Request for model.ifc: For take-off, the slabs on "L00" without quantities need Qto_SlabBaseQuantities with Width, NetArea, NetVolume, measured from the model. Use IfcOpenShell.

First a look at what the model holds.

```python
import ifcopenshell
import ifcopenshell.util.element
import ifcopenshell.util.unit

model = ifcopenshell.open("model.ifc")
print(model.schema)
for unit_type in ("LENGTHUNIT", "AREAUNIT", "VOLUMEUNIT"):
    print(unit_type, ifcopenshell.util.unit.calculate_unit_scale(model, unit_type))
storey = next(s for s in model.by_type("IfcBuildingStorey") if s.Name == "L00")
slabs = [e for e in ifcopenshell.util.element.get_decomposition(storey) if e.is_a("IfcSlab")]
for e in sorted(slabs, key=lambda e: e.id()):
    print(e.id(), e.is_a(), e.Name, list(ifcopenshell.util.element.get_psets(e, qtos_only=True)), sep=" | ")
```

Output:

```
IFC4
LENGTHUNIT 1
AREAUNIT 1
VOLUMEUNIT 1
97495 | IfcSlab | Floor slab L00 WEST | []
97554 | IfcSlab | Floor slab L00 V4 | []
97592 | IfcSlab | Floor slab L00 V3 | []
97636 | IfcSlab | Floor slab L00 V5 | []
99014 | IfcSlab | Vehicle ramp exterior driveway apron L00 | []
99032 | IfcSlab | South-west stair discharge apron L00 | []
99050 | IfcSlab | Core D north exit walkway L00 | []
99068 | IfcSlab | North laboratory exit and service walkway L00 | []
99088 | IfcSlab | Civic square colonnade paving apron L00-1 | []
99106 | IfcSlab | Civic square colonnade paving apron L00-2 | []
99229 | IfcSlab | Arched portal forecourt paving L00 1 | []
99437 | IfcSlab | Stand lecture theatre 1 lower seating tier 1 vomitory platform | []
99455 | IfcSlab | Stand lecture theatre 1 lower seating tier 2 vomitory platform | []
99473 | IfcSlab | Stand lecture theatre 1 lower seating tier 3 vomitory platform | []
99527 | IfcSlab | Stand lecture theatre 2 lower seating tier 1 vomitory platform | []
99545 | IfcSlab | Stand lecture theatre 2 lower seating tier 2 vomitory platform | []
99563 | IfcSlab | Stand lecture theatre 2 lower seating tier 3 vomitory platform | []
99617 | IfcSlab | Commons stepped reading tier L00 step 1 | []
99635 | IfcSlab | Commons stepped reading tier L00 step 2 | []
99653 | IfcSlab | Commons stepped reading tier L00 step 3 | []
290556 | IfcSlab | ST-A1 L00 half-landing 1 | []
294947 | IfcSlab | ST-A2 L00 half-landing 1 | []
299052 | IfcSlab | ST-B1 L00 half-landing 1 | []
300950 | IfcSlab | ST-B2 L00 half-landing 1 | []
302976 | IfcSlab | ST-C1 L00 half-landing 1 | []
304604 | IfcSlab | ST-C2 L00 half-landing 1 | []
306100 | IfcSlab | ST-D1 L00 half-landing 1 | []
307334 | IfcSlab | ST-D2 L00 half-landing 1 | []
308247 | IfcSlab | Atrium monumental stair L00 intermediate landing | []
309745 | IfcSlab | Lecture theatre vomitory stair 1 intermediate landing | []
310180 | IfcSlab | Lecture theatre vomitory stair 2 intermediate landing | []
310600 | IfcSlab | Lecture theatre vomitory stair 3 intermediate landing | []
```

```python
import ifcopenshell
import ifcopenshell.api.pset
import ifcopenshell.geom
import ifcopenshell.util.element
import ifcopenshell.util.shape
import ifcopenshell.util.unit

model = ifcopenshell.open("model.ifc")
unit_scale = ifcopenshell.util.unit.calculate_unit_scale(model)
area_scale = ifcopenshell.util.unit.calculate_unit_scale(model, "AREAUNIT")
volume_scale = ifcopenshell.util.unit.calculate_unit_scale(model, "VOLUMEUNIT")
settings = ifcopenshell.geom.settings()

storey = next(s for s in model.by_type("IfcBuildingStorey") if s.Name == "L00")
slabs = [e for e in ifcopenshell.util.element.get_decomposition(storey) if e.is_a("IfcSlab")]

for e in sorted(slabs, key=lambda e: e.id()):
    if ifcopenshell.util.element.get_psets(e, qtos_only=True, should_inherit=False):
        continue
    # Geometry comes back in metres, in the element's own axes.
    shape = ifcopenshell.geom.create_shape(settings, e)
    values = {
        "Width": ifcopenshell.util.shape.get_z(shape.geometry) / unit_scale,
        "NetArea": ifcopenshell.util.shape.get_footprint_area(shape.geometry) / area_scale,
        "NetVolume": ifcopenshell.util.shape.get_volume(shape.geometry) / volume_scale,
    }
    qto = ifcopenshell.api.pset.add_qto(model, product=e, name="Qto_SlabBaseQuantities")
    ifcopenshell.api.pset.edit_qto(model, qto=qto, properties=values)
    print(e.id(), {k: round(v, 3) for k, v in values.items()})

model.write("model_edited.ifc")
```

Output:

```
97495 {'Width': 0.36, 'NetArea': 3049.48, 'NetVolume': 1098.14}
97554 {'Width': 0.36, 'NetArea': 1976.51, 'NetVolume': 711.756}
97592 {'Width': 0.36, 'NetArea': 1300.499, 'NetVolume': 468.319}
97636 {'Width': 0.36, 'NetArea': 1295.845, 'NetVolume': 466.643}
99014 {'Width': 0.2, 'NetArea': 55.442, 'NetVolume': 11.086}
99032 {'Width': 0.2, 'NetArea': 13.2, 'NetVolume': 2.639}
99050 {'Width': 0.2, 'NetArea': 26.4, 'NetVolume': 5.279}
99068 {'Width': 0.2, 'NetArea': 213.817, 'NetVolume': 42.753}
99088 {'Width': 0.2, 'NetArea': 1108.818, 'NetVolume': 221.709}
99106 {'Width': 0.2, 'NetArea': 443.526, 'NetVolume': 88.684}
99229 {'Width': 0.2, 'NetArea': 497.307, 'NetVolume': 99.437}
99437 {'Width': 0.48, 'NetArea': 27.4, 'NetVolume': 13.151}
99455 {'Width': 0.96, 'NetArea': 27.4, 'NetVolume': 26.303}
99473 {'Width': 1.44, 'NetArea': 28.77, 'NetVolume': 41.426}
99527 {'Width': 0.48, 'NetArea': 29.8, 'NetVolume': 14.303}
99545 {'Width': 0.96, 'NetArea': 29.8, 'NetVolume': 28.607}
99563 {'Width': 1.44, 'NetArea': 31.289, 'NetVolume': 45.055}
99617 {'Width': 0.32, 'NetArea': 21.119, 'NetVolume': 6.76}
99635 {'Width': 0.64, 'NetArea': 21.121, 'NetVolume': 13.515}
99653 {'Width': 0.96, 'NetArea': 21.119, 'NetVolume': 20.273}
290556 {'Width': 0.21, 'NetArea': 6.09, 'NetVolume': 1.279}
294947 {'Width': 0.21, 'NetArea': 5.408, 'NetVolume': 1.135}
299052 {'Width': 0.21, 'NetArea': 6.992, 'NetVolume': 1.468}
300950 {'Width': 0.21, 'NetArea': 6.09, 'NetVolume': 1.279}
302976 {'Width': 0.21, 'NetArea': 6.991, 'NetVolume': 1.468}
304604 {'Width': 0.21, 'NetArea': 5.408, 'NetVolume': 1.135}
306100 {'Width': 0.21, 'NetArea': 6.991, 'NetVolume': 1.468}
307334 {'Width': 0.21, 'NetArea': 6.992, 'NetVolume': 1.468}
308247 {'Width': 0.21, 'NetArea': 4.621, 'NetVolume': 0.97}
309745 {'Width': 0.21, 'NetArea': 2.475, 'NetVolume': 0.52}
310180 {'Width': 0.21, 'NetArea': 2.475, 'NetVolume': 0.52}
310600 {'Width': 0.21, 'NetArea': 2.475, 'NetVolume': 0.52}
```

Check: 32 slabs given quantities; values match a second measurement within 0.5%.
